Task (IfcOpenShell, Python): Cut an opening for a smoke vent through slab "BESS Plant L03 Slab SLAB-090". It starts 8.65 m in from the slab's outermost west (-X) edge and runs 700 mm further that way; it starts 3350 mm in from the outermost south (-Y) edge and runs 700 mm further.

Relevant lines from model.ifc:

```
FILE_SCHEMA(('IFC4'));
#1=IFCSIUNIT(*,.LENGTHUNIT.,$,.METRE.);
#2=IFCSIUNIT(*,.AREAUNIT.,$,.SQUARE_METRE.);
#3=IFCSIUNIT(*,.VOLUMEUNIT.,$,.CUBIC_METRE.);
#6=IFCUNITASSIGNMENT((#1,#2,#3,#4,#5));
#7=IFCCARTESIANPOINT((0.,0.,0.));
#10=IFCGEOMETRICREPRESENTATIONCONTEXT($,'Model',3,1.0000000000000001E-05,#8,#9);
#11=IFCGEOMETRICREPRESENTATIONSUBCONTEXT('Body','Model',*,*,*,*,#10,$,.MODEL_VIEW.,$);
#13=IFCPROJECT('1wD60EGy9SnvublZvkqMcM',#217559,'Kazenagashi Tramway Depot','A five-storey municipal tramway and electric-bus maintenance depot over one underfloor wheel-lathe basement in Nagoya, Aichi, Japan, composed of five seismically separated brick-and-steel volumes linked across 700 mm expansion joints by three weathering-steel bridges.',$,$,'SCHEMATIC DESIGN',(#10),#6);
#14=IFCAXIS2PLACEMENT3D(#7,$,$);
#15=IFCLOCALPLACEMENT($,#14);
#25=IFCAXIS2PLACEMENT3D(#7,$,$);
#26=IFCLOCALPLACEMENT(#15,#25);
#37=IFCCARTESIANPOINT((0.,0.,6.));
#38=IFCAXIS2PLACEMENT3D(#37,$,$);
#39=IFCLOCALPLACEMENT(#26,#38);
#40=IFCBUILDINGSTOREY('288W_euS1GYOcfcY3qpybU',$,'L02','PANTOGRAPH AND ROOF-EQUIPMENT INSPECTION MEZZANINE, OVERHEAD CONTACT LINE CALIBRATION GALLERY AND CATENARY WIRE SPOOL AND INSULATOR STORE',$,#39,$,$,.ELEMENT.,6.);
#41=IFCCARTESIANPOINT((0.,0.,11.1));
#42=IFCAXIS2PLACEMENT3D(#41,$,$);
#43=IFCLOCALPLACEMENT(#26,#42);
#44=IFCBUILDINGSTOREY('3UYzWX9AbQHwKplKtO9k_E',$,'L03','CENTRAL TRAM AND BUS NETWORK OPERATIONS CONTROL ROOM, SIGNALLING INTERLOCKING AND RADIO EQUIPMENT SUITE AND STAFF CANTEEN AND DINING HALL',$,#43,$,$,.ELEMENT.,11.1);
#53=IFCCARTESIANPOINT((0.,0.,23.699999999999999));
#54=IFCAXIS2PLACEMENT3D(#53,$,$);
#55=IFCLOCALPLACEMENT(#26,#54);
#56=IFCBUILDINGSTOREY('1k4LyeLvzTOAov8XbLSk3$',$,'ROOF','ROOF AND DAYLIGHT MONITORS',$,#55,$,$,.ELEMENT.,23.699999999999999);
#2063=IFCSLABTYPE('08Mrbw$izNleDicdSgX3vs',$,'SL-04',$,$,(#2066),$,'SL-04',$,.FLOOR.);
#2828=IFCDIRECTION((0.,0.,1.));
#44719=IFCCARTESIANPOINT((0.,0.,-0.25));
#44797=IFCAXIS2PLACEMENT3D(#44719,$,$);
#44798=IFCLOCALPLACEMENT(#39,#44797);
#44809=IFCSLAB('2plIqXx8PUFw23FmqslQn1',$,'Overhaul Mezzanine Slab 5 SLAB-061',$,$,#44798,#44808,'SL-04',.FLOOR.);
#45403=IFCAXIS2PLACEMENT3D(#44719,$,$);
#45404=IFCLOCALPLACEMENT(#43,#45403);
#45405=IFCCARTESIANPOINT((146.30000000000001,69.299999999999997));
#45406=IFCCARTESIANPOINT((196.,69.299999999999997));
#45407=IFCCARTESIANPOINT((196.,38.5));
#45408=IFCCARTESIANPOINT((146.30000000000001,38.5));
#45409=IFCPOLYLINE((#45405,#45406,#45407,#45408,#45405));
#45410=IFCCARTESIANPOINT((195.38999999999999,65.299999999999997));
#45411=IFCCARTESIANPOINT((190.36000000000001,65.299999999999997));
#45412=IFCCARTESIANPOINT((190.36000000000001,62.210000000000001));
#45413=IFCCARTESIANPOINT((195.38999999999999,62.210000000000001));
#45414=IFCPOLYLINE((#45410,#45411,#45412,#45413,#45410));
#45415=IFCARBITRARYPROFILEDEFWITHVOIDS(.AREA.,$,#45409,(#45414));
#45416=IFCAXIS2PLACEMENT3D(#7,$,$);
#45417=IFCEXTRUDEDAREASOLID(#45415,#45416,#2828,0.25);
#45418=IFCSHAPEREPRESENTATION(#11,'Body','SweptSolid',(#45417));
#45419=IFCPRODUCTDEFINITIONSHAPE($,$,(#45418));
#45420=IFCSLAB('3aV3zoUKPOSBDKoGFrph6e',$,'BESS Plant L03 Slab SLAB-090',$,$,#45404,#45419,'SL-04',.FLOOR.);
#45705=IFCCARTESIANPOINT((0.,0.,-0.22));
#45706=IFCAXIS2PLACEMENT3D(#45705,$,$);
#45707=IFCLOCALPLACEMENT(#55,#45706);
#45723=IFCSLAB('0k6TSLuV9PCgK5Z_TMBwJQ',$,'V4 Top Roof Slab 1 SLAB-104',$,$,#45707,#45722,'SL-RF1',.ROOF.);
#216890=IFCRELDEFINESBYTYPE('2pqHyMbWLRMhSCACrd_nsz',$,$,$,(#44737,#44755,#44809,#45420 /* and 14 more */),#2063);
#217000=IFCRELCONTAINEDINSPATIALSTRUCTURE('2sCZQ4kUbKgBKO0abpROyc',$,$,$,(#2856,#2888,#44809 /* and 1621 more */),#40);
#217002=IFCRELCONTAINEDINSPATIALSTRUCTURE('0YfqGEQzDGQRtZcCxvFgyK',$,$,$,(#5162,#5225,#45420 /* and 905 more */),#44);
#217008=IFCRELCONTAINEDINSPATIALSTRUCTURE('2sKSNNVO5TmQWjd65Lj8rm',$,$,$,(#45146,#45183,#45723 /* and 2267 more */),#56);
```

```python
import numpy as np
import ifcopenshell
import ifcopenshell.api.feature
import ifcopenshell.api.geometry
import ifcopenshell.api.root
import ifcopenshell.geom
import ifcopenshell.util.placement
import ifcopenshell.util.representation
import ifcopenshell.util.shape
import ifcopenshell.util.unit

model = ifcopenshell.open("model.ifc")
unit_scale = ifcopenshell.util.unit.calculate_unit_scale(model)
settings = ifcopenshell.geom.settings()


def volume(element):
    """Net volume in cubic metres, openings subtracted."""
    shape = ifcopenshell.geom.create_shape(settings, element)
    return ifcopenshell.util.shape.get_volume(shape.geometry)


slab = model.by_id(45420)
before = volume(slab)

# Extent in the slab's own axes, in metres. The edges named are its -X and -Y sides.
slab_shape = ifcopenshell.geom.create_shape(settings, slab)
vertices = ifcopenshell.util.shape.get_vertices(slab_shape.geometry)
x_min, y_min, bottom = vertices.min(axis=0)
top = vertices[:, 2].max()

opening = ifcopenshell.api.root.create_entity(model, ifc_class="IfcOpeningElement", name="Smoke vent opening", predefined_type="OPENING")
context = ifcopenshell.util.representation.get_context(model, "Model", "Body", "MODEL_VIEW")
width, depth = 0.7, 0.7
outline = [(0.0, 0.0), (width, 0.0), (width, depth), (0.0, depth), (0.0, 0.0)]
# Overshoot both faces by 50 mm so the cut is clean.
shape = ifcopenshell.api.geometry.add_slab_representation(
    model, context=context, depth=top - bottom + 0.1, polyline=outline
)
ifcopenshell.api.geometry.assign_representation(model, product=opening, representation=shape)

matrix = ifcopenshell.util.placement.get_local_placement(slab.ObjectPlacement)
matrix[:, 3] = matrix @ np.append(np.array([x_min + 8.65, y_min + 3.35, bottom - 0.05]) / unit_scale, 1.0)
ifcopenshell.api.geometry.edit_object_placement(model, product=opening, matrix=matrix, is_si=False)
ifcopenshell.api.feature.add_feature(model, feature=opening, element=slab)

after = volume(slab)

print(f"slab volume {before:.3f} -> {after:.3f} m3")

model.write("model-out.ifc")
```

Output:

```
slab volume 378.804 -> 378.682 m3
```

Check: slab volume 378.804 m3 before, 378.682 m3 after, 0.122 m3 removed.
